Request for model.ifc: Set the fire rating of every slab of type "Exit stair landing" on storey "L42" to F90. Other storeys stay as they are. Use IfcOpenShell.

First a look at what the model holds.

```python
import ifcopenshell
import ifcopenshell.util.element

model = ifcopenshell.open("model.ifc")
print(model.schema)
storey = next(s for s in model.by_type("IfcBuildingStorey") if s.Name == "L42")
slabs = [e for e in ifcopenshell.util.element.get_decomposition(storey) if e.is_a("IfcSlab")]
seen = {}
for e in slabs:
    element_type = ifcopenshell.util.element.get_type(e)
    key = (element_type.Name if element_type != e and element_type else None, ifcopenshell.util.element.get_pset(e, "Pset_SlabCommon", "FireRating"))
    seen[key] = seen.get(key, 0) + 1
for (name, value), count in sorted(seen.items(), key=str):
    print(count, "x", name, "|", value)
```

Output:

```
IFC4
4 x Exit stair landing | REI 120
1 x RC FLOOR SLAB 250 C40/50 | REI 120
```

```python
import ifcopenshell
import ifcopenshell.api.pset
import ifcopenshell.util.element

model = ifcopenshell.open("model.ifc")

storey = next(s for s in model.by_type("IfcBuildingStorey") if s.Name == "L42")
slabs = [e for e in ifcopenshell.util.element.get_decomposition(storey) if e.is_a("IfcSlab")]

count = 0
for e in slabs:
    element_type = ifcopenshell.util.element.get_type(e)
    if element_type in (None, e) or element_type.Name != "Exit stair landing":
        continue
    found = ifcopenshell.util.element.get_pset(e, "Pset_SlabCommon", should_inherit=False)
    if found:
        pset = model.by_id(found["id"])
        if len(ifcopenshell.util.element.get_elements_by_pset(pset)) > 1:
            pset = ifcopenshell.api.pset.unshare_pset(model, products=[e], pset=pset)[0]
    else:
        pset = ifcopenshell.api.pset.add_pset(model, product=e, name="Pset_SlabCommon")
    ifcopenshell.api.pset.edit_pset(model, pset=pset, properties={"FireRating": "F90"})
    count += 1

print(count, "slabs updated")

model.write("model_v2.ifc")
```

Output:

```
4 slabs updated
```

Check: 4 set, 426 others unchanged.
